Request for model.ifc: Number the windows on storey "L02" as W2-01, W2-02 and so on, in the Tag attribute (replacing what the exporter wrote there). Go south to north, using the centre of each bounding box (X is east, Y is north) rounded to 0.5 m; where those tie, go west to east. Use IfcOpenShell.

First a look at what the model holds.

```python
import ifcopenshell
import ifcopenshell.util.element
import ifcopenshell.util.placement

model = ifcopenshell.open("model.ifc")
print(model.schema)
storey = next(s for s in model.by_type("IfcBuildingStorey") if s.Name == "L02")
windows = [e for e in ifcopenshell.util.element.get_decomposition(storey) if e.is_a("IfcWindow")]
for e in sorted(windows, key=lambda e: e.id()):
    origin = ifcopenshell.util.placement.get_local_placement(e.ObjectPlacement)[:3, 3]
    print(e.id(), e.Tag, e.Name, origin.round(2) + 0.0, sep=" | ")
```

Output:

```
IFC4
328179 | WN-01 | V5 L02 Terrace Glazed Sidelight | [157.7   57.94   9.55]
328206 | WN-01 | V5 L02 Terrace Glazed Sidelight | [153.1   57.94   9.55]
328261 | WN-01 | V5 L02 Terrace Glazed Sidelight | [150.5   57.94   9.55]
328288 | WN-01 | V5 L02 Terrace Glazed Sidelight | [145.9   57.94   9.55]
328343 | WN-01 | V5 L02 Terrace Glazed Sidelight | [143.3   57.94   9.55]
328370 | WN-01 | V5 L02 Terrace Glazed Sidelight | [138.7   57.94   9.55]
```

```python
import ifcopenshell
import ifcopenshell.geom
import ifcopenshell.util.element
import ifcopenshell.util.shape

model = ifcopenshell.open("model.ifc")
settings = ifcopenshell.geom.settings()
settings.set("use-world-coords", True)


def centre(element):
    shape = ifcopenshell.geom.create_shape(settings, element)
    return ifcopenshell.util.shape.get_bbox_centroid(shape.geometry)


storey = next(s for s in model.by_type("IfcBuildingStorey") if s.Name == "L02")
windows = [e for e in ifcopenshell.util.element.get_decomposition(storey) if e.is_a("IfcWindow")]

# Insertion points can sit at a corner or the storey origin, so sort by the geometry (in metres).
centres = {e: centre(e) for e in windows}
windows.sort(key=lambda e: (round(centres[e][1] / 0.5), centres[e][0]))

for i, e in enumerate(windows, start=1):
    number = f"W2-{i:02d}"
    e.Tag = number
    print(e.id(), number)

model.write("model_v2.ifc")
```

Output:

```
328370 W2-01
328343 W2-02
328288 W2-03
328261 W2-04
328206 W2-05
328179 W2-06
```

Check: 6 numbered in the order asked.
